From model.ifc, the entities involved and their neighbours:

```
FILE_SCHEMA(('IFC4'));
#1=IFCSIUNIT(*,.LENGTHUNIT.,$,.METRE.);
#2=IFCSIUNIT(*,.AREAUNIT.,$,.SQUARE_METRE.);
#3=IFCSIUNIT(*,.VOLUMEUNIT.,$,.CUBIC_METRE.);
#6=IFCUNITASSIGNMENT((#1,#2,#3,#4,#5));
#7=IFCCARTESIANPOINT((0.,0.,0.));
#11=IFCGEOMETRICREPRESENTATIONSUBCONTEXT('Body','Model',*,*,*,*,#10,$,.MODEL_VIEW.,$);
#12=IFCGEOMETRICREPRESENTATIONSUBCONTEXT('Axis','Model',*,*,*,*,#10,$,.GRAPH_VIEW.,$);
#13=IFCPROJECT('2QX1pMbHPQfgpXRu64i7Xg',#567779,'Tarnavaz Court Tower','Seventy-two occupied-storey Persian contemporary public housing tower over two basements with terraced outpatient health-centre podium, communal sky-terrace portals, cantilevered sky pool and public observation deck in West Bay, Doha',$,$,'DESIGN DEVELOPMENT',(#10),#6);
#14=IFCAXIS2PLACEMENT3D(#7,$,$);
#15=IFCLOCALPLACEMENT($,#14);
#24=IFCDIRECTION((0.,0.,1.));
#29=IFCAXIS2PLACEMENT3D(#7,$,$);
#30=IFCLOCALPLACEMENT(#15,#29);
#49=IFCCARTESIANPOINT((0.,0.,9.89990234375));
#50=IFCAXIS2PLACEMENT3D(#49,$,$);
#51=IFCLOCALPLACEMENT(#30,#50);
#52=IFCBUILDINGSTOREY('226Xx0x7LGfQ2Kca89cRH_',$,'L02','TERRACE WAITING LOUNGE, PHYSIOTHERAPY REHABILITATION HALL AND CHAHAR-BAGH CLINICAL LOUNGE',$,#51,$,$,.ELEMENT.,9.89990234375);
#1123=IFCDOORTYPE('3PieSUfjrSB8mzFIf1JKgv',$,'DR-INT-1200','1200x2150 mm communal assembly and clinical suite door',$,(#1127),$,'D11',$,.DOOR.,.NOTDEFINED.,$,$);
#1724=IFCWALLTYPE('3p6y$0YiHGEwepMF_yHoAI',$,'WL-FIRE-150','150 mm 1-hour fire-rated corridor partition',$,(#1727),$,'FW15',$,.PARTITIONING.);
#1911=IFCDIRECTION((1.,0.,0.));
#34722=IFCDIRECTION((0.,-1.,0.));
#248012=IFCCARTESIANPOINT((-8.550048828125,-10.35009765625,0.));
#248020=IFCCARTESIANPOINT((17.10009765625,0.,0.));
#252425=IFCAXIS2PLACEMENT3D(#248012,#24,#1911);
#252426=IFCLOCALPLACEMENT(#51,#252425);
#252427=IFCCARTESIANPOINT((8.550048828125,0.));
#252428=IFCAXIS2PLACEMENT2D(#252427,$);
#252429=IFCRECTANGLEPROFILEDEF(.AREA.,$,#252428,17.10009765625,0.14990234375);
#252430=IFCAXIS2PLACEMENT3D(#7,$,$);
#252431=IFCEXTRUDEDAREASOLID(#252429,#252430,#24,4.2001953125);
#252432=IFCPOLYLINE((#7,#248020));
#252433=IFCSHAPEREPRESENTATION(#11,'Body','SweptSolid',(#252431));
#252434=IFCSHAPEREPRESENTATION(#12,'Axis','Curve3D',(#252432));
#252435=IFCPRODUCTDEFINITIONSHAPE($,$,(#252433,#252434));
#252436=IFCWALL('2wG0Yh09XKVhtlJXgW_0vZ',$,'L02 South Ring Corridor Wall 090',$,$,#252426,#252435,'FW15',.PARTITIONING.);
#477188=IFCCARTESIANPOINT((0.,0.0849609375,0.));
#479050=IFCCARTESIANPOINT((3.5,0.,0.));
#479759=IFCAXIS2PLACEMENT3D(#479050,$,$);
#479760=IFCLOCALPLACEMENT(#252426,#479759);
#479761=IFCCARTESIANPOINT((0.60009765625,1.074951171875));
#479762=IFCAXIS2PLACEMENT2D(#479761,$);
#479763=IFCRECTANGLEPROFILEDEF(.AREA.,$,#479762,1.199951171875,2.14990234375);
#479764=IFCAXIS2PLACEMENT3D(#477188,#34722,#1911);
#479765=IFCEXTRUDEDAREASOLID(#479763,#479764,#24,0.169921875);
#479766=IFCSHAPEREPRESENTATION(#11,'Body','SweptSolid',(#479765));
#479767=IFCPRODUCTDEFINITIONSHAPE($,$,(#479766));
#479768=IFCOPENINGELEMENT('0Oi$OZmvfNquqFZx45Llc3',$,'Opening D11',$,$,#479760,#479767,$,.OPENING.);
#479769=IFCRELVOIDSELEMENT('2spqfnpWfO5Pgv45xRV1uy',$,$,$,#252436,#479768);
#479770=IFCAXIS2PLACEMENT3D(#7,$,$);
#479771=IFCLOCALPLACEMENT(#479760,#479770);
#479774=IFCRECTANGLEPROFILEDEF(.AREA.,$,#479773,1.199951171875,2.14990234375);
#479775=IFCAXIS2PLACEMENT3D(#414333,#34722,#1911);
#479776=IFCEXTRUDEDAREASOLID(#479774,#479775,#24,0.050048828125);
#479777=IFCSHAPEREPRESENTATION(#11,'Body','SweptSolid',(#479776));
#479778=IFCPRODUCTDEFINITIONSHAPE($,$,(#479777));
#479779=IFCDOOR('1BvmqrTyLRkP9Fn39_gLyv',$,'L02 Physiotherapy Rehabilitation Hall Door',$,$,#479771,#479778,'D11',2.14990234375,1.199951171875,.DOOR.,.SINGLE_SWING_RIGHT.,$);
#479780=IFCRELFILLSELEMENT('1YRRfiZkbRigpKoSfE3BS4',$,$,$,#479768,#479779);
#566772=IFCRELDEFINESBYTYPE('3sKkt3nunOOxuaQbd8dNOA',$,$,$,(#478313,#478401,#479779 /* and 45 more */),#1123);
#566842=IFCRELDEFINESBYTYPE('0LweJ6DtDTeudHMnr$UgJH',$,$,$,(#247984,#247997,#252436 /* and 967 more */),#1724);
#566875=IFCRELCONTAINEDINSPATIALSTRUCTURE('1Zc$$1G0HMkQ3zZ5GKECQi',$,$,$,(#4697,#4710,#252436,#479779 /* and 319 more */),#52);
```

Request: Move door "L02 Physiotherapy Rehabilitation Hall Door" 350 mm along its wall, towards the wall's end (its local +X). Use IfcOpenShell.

```python
import ifcopenshell
import ifcopenshell.api.geometry
import ifcopenshell.util.placement

model = ifcopenshell.open("model.ifc")

door = model.by_id(479779)
opening = door.FillsVoids[0].RelatingOpeningElement
wall = opening.VoidsElements[0].RelatingBuildingElement

wall_matrix = ifcopenshell.util.placement.get_local_placement(wall.ObjectPlacement)
shift = wall_matrix[:3, 0] * 0.35
before = ifcopenshell.util.placement.get_local_placement(door.ObjectPlacement)[:3, 3].copy()

# The door is placed relative to its opening, so it follows when the opening moves.
matrix = ifcopenshell.util.placement.get_local_placement(opening.ObjectPlacement)
matrix[:3, 3] += shift
ifcopenshell.api.geometry.edit_object_placement(
    model, product=opening, matrix=matrix, is_si=False, should_transform_children=True
)

after = ifcopenshell.util.placement.get_local_placement(door.ObjectPlacement)[:3, 3]
print("door moved by", (after - before).round(3) + 0.0)

model.write("model_edited.ifc")
```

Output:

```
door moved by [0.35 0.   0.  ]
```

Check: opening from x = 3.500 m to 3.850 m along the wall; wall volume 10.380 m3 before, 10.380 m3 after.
